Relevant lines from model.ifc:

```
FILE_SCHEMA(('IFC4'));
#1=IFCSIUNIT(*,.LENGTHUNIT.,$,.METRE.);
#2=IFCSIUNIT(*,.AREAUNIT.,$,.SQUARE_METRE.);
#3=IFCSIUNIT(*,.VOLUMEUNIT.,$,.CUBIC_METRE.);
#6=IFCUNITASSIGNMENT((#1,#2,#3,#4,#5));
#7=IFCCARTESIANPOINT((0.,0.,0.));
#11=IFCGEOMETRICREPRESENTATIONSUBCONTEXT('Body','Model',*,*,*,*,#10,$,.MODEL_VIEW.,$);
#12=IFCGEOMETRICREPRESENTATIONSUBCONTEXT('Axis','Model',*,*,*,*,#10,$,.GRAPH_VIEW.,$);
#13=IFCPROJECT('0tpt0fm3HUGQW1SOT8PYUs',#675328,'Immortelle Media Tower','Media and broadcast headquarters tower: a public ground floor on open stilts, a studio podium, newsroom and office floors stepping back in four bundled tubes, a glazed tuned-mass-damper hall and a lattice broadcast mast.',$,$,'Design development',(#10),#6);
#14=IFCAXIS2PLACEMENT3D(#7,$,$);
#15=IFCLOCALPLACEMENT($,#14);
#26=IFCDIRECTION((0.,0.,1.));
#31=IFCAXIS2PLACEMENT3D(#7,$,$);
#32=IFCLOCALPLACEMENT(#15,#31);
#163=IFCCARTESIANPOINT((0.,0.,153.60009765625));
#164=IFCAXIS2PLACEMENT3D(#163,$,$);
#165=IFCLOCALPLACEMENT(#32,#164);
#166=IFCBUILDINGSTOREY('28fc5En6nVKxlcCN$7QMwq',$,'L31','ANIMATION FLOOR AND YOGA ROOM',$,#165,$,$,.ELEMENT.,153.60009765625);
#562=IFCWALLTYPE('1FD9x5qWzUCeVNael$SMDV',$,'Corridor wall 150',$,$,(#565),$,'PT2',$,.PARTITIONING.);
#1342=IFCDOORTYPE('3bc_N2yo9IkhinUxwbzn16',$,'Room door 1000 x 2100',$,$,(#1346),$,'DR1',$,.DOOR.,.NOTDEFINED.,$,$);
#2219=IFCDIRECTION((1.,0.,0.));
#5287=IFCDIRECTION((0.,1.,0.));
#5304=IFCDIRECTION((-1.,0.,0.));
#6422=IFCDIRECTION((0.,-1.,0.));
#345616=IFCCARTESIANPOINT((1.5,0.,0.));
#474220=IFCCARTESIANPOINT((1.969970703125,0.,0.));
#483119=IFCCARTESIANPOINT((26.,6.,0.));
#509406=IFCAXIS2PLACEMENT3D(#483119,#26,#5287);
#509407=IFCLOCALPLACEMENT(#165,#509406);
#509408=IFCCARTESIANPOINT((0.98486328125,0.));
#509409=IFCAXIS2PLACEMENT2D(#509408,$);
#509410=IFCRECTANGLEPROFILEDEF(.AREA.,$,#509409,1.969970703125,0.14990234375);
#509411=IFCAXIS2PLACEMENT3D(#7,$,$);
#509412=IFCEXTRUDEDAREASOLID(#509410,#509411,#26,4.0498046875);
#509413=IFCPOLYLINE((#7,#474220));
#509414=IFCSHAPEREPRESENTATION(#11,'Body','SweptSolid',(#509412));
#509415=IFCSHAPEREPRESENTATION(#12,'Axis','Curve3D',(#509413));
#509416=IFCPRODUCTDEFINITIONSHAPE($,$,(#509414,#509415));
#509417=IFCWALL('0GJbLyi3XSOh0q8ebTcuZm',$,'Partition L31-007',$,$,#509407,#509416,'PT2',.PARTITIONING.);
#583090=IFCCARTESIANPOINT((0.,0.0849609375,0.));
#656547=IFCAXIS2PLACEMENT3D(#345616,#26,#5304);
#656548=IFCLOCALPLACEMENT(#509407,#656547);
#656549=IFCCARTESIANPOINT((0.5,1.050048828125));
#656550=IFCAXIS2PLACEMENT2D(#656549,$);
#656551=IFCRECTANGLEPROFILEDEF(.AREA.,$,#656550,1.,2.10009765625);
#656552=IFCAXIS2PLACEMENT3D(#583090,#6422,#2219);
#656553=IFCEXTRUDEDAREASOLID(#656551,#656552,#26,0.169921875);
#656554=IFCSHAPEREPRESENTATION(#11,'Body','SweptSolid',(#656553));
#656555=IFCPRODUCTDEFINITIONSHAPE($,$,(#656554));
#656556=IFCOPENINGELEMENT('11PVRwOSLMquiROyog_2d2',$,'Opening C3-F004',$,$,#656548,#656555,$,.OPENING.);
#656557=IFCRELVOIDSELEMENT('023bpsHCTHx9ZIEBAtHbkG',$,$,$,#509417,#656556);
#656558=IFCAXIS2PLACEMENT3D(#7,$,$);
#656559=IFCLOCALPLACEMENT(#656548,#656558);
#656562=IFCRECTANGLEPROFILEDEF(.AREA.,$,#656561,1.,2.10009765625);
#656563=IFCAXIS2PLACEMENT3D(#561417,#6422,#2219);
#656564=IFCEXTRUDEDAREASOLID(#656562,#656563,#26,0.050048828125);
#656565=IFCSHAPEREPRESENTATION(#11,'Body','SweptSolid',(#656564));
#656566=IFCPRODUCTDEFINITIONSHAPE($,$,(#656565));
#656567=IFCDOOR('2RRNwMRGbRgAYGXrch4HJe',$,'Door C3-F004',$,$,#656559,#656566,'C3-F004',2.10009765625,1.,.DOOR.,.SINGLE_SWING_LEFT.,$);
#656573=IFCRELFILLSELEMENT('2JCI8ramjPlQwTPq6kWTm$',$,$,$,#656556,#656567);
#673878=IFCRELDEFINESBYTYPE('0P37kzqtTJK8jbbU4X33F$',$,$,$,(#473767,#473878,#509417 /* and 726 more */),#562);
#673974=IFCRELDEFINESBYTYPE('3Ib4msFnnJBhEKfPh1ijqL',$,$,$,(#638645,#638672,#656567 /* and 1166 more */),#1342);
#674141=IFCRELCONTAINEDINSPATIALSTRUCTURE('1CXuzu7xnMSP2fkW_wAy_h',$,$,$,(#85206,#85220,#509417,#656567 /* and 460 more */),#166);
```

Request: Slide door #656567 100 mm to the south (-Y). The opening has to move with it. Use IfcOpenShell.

```python
import ifcopenshell
import ifcopenshell.api.geometry
import ifcopenshell.util.placement
import ifcopenshell.util.unit

model = ifcopenshell.open("model.ifc")
unit_scale = ifcopenshell.util.unit.calculate_unit_scale(model)

door = model.by_guid("2RRNwMRGbRgAYGXrch4HJe")
opening = door.FillsVoids[0].RelatingOpeningElement
wall = opening.VoidsElements[0].RelatingBuildingElement

wall_matrix = ifcopenshell.util.placement.get_local_placement(wall.ObjectPlacement)
shift = wall_matrix[:3, 0] * -0.1 / unit_scale
before = ifcopenshell.util.placement.get_local_placement(door.ObjectPlacement)[:3, 3].copy()

# The door is placed relative to its opening, so it follows when the opening moves.
matrix = ifcopenshell.util.placement.get_local_placement(opening.ObjectPlacement)
matrix[:3, 3] += shift
ifcopenshell.api.geometry.edit_object_placement(
    model, product=opening, matrix=matrix, is_si=False, should_transform_children=True
)

after = ifcopenshell.util.placement.get_local_placement(door.ObjectPlacement)[:3, 3]
print("door moved by", (after - before).round(3) + 0.0)

model.write("model-out.ifc")
```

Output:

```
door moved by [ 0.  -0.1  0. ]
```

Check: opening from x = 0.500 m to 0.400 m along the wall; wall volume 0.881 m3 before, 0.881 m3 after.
